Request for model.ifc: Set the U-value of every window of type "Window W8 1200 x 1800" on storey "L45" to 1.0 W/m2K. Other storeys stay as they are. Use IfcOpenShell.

First a look at what the model holds.

```python
import ifcopenshell
import ifcopenshell.util.element

model = ifcopenshell.open("model.ifc")
print(model.schema)
storey = next(s for s in model.by_type("IfcBuildingStorey") if s.Name == "L45")
windows = [e for e in ifcopenshell.util.element.get_decomposition(storey) if e.is_a("IfcWindow")]
seen = {}
for e in windows:
    element_type = ifcopenshell.util.element.get_type(e)
    key = (element_type.Name if element_type != e and element_type else None, ifcopenshell.util.element.get_pset(e, "Pset_WindowCommon", "ThermalTransmittance"))
    seen[key] = seen.get(key, 0) + 1
for (name, value), count in sorted(seen.items(), key=str):
    print(count, "x", name, "|", value)
```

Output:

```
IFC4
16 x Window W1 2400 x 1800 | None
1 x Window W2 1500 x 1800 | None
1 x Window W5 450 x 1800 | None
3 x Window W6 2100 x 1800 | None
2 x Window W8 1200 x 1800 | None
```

```python
import ifcopenshell
import ifcopenshell.api.pset
import ifcopenshell.util.element

model = ifcopenshell.open("model.ifc")

storey = next(s for s in model.by_type("IfcBuildingStorey") if s.Name == "L45")
windows = [e for e in ifcopenshell.util.element.get_decomposition(storey) if e.is_a("IfcWindow")]

count = 0
for e in windows:
    element_type = ifcopenshell.util.element.get_type(e)
    if element_type in (None, e) or element_type.Name != "Window W8 1200 x 1800":
        continue
    found = ifcopenshell.util.element.get_pset(e, "Pset_WindowCommon", should_inherit=False)
    if found:
        pset = model.by_id(found["id"])
        if len(ifcopenshell.util.element.get_elements_by_pset(pset)) > 1:
            pset = ifcopenshell.api.pset.unshare_pset(model, products=[e], pset=pset)[0]
    else:
        pset = ifcopenshell.api.pset.add_pset(model, product=e, name="Pset_WindowCommon")
    ifcopenshell.api.pset.edit_pset(model, pset=pset, properties={"ThermalTransmittance": 1.0})
    count += 1

print(count, "windows updated")

model.write("model-out.ifc")
```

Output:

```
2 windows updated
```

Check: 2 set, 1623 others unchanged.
